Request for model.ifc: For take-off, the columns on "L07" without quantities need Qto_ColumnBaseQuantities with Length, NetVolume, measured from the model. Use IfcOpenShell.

First a look at what the model holds.

```python
import ifcopenshell
import ifcopenshell.util.element
import ifcopenshell.util.unit

model = ifcopenshell.open("model.ifc")
print(model.schema)
for unit_type in ("LENGTHUNIT", "AREAUNIT", "VOLUMEUNIT"):
    print(unit_type, ifcopenshell.util.unit.calculate_unit_scale(model, unit_type))
storey = next(s for s in model.by_type("IfcBuildingStorey") if s.Name == "L07")
columns = [e for e in ifcopenshell.util.element.get_decomposition(storey) if e.is_a("IfcColumn")]
for e in sorted(columns, key=lambda e: e.id()):
    print(e.id(), e.is_a(), e.Name, list(ifcopenshell.util.element.get_psets(e, qtos_only=True)), sep=" | ")
```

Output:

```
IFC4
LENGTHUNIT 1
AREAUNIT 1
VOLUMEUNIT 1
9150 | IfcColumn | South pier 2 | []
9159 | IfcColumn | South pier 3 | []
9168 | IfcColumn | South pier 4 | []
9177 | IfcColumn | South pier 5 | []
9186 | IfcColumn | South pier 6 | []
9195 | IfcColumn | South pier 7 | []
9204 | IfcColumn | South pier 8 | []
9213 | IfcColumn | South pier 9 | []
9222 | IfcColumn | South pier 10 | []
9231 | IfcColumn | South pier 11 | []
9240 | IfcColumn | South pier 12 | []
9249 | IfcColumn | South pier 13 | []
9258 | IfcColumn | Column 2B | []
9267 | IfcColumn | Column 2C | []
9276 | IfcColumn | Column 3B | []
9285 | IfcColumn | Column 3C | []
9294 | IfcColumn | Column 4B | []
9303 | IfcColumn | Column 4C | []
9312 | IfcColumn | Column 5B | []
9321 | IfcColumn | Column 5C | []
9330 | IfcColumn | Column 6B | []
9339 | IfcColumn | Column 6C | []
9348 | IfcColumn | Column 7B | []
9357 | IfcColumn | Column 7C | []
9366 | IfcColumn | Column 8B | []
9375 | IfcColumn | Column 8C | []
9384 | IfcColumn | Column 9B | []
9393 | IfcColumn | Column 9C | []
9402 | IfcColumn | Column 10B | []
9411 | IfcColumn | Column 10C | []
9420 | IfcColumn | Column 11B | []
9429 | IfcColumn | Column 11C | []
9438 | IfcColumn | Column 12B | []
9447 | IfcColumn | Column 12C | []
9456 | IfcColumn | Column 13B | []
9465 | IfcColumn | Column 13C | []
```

```python
import ifcopenshell
import ifcopenshell.api.pset
import ifcopenshell.geom
import ifcopenshell.util.element
import ifcopenshell.util.shape
import ifcopenshell.util.unit

model = ifcopenshell.open("model.ifc")
unit_scale = ifcopenshell.util.unit.calculate_unit_scale(model)
volume_scale = ifcopenshell.util.unit.calculate_unit_scale(model, "VOLUMEUNIT")
settings = ifcopenshell.geom.settings()

storey = next(s for s in model.by_type("IfcBuildingStorey") if s.Name == "L07")
columns = [e for e in ifcopenshell.util.element.get_decomposition(storey) if e.is_a("IfcColumn")]

for e in sorted(columns, key=lambda e: e.id()):
    if ifcopenshell.util.element.get_psets(e, qtos_only=True, should_inherit=False):
        continue
    # Geometry comes back in metres, in the element's own axes.
    shape = ifcopenshell.geom.create_shape(settings, e)
    values = {
        "Length": ifcopenshell.util.shape.get_z(shape.geometry) / unit_scale,
        "NetVolume": ifcopenshell.util.shape.get_volume(shape.geometry) / volume_scale,
    }
    qto = ifcopenshell.api.pset.add_qto(model, product=e, name="Qto_ColumnBaseQuantities")
    ifcopenshell.api.pset.edit_qto(model, qto=qto, properties=values)
    print(e.id(), {k: round(v, 3) for k, v in values.items()})

model.write("model_v2.ifc")
```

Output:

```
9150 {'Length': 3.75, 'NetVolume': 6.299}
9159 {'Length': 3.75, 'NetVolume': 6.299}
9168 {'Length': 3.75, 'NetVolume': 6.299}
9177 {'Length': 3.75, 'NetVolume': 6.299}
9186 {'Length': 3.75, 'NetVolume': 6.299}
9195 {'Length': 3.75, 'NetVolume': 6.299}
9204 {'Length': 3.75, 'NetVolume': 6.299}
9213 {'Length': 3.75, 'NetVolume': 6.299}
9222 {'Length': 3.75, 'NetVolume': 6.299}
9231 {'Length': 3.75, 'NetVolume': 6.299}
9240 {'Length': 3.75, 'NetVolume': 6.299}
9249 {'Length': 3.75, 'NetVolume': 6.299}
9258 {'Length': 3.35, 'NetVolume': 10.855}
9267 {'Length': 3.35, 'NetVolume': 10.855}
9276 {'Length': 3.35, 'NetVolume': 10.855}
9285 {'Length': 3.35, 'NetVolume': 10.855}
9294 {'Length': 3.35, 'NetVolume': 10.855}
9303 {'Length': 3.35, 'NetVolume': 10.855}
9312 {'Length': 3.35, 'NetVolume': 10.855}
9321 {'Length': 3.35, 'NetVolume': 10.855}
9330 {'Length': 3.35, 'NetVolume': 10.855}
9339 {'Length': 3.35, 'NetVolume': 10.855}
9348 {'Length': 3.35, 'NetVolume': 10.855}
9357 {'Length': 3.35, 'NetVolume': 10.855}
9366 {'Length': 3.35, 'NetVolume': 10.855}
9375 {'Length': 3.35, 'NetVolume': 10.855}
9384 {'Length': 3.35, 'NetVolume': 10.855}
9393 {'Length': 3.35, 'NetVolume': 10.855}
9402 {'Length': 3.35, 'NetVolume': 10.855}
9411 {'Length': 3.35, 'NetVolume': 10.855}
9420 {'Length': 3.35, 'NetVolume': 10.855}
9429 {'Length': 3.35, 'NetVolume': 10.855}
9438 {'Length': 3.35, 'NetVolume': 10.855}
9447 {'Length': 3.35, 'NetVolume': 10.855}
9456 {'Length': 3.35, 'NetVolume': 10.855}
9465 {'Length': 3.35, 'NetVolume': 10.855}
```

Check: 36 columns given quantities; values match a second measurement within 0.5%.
